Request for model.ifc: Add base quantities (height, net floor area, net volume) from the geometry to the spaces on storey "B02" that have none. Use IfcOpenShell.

First a look at what the model holds.

```python
import ifcopenshell
import ifcopenshell.util.element
import ifcopenshell.util.unit

model = ifcopenshell.open("model.ifc")
print(model.schema)
for unit_type in ("LENGTHUNIT", "AREAUNIT", "VOLUMEUNIT"):
    print(unit_type, ifcopenshell.util.unit.calculate_unit_scale(model, unit_type))
storey = next(s for s in model.by_type("IfcBuildingStorey") if s.Name == "B02")
spaces = [e for e in ifcopenshell.util.element.get_decomposition(storey) if e.is_a("IfcSpace")]
for e in sorted(spaces, key=lambda e: e.id()):
    print(e.id(), e.is_a(), e.Name, list(ifcopenshell.util.element.get_psets(e, qtos_only=True)), sep=" | ")
```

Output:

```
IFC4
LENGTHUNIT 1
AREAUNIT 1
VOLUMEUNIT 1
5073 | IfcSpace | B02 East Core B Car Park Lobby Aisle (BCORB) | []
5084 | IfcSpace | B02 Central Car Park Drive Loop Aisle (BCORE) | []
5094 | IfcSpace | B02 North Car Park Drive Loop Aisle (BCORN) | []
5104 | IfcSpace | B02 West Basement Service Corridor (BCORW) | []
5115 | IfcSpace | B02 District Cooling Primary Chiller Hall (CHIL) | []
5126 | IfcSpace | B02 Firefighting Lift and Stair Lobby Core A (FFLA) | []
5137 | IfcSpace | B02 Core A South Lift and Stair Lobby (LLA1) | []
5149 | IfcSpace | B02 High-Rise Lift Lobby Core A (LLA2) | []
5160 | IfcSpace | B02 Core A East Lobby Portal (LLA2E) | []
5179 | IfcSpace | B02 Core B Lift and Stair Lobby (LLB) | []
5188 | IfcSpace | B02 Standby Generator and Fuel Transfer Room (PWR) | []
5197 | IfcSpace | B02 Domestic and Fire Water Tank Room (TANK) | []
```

```python
import ifcopenshell
import ifcopenshell.api.pset
import ifcopenshell.geom
import ifcopenshell.util.element
import ifcopenshell.util.shape
import ifcopenshell.util.unit

model = ifcopenshell.open("model.ifc")
unit_scale = ifcopenshell.util.unit.calculate_unit_scale(model)
area_scale = ifcopenshell.util.unit.calculate_unit_scale(model, "AREAUNIT")
volume_scale = ifcopenshell.util.unit.calculate_unit_scale(model, "VOLUMEUNIT")
settings = ifcopenshell.geom.settings()

storey = next(s for s in model.by_type("IfcBuildingStorey") if s.Name == "B02")
spaces = [e for e in ifcopenshell.util.element.get_decomposition(storey) if e.is_a("IfcSpace")]

for e in sorted(spaces, key=lambda e: e.id()):
    if ifcopenshell.util.element.get_psets(e, qtos_only=True, should_inherit=False):
        continue
    # Geometry comes back in metres, in the element's own axes.
    shape = ifcopenshell.geom.create_shape(settings, e)
    values = {
        "Height": ifcopenshell.util.shape.get_z(shape.geometry) / unit_scale,
        "NetFloorArea": ifcopenshell.util.shape.get_footprint_area(shape.geometry) / area_scale,
        "NetVolume": ifcopenshell.util.shape.get_volume(shape.geometry) / volume_scale,
    }
    qto = ifcopenshell.api.pset.add_qto(model, product=e, name="Qto_SpaceBaseQuantities")
    ifcopenshell.api.pset.edit_qto(model, qto=qto, properties=values)
    print(e.id(), {k: round(v, 3) for k, v in values.items()})

model.write("model_rev.ifc")
```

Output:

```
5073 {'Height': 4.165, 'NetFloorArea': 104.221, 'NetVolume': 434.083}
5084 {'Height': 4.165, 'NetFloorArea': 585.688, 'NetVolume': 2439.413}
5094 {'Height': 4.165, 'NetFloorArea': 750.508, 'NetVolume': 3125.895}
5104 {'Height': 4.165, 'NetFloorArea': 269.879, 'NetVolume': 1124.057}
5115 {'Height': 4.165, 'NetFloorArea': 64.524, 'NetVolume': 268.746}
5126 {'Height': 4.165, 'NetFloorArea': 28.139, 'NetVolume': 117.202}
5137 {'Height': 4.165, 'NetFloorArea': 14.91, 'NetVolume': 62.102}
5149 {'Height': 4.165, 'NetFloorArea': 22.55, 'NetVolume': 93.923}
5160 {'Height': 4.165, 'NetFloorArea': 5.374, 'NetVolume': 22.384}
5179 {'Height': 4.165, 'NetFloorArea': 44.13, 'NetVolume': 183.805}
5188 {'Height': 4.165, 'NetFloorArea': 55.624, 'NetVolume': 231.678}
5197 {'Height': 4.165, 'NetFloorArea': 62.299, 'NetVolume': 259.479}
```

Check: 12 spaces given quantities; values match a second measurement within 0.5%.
